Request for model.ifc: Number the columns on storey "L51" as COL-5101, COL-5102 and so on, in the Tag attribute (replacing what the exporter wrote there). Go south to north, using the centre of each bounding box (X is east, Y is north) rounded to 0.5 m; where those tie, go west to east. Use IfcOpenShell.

First a look at what the model holds.

```python
import ifcopenshell
import ifcopenshell.util.element
import ifcopenshell.util.placement

model = ifcopenshell.open("model.ifc")
print(model.schema)
storey = next(s for s in model.by_type("IfcBuildingStorey") if s.Name == "L51")
columns = [e for e in ifcopenshell.util.element.get_decomposition(storey) if e.is_a("IfcColumn")]
for e in sorted(columns, key=lambda e: e.id()):
    origin = ifcopenshell.util.placement.get_local_placement(e.ObjectPlacement)[:3, 3]
    print(e.id(), e.Tag, e.Name, origin.round(2) + 0.0, sep=" | ")
```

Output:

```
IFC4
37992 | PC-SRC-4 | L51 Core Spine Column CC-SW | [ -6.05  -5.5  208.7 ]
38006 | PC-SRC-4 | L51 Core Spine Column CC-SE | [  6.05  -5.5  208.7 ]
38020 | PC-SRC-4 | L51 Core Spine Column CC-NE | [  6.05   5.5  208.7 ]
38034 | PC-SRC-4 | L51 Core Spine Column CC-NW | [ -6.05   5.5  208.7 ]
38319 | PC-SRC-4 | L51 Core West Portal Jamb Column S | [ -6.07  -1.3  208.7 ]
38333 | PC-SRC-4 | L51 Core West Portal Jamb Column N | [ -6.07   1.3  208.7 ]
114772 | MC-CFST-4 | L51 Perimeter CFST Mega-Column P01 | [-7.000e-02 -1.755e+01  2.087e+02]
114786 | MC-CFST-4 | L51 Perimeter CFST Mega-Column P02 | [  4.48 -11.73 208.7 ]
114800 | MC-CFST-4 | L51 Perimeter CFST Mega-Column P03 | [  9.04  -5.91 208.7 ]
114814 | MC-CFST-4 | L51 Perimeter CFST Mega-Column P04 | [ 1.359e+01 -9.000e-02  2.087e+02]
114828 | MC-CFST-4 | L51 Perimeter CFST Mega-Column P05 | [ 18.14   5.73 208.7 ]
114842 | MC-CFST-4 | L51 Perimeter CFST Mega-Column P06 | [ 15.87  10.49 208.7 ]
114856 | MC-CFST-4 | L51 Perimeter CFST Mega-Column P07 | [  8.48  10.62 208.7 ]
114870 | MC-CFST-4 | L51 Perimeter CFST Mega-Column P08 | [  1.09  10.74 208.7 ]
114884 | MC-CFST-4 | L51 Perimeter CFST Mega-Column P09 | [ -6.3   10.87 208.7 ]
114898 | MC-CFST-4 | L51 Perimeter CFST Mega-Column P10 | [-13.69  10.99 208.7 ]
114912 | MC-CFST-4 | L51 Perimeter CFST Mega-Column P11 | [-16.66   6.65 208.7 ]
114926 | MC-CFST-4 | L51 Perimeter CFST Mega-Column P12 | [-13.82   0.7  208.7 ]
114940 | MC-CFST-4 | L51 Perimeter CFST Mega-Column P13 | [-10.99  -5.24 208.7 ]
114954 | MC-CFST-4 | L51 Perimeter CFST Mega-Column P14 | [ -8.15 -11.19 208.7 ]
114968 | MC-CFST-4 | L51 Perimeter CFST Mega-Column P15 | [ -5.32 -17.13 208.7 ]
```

```python
import ifcopenshell
import ifcopenshell.geom
import ifcopenshell.util.element
import ifcopenshell.util.shape

model = ifcopenshell.open("model.ifc")
settings = ifcopenshell.geom.settings()
settings.set("use-world-coords", True)


def centre(element):
    shape = ifcopenshell.geom.create_shape(settings, element)
    return ifcopenshell.util.shape.get_bbox_centroid(shape.geometry)


storey = next(s for s in model.by_type("IfcBuildingStorey") if s.Name == "L51")
columns = [e for e in ifcopenshell.util.element.get_decomposition(storey) if e.is_a("IfcColumn")]

# Insertion points can sit at a corner or the storey origin, so sort by the geometry (in metres).
centres = {e: centre(e) for e in columns}
columns.sort(key=lambda e: (round(centres[e][1] / 0.5), centres[e][0]))

for i, e in enumerate(columns, start=1):
    number = f"COL-51{i:02d}"
    e.Tag = number
    print(e.id(), number)

model.write("model_updated.ifc")
```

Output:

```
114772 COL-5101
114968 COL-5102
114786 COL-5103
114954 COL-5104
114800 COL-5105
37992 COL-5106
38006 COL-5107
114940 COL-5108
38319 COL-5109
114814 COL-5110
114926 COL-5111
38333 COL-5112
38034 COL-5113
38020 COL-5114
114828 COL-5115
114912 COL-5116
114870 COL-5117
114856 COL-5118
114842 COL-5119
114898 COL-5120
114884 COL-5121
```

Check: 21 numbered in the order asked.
